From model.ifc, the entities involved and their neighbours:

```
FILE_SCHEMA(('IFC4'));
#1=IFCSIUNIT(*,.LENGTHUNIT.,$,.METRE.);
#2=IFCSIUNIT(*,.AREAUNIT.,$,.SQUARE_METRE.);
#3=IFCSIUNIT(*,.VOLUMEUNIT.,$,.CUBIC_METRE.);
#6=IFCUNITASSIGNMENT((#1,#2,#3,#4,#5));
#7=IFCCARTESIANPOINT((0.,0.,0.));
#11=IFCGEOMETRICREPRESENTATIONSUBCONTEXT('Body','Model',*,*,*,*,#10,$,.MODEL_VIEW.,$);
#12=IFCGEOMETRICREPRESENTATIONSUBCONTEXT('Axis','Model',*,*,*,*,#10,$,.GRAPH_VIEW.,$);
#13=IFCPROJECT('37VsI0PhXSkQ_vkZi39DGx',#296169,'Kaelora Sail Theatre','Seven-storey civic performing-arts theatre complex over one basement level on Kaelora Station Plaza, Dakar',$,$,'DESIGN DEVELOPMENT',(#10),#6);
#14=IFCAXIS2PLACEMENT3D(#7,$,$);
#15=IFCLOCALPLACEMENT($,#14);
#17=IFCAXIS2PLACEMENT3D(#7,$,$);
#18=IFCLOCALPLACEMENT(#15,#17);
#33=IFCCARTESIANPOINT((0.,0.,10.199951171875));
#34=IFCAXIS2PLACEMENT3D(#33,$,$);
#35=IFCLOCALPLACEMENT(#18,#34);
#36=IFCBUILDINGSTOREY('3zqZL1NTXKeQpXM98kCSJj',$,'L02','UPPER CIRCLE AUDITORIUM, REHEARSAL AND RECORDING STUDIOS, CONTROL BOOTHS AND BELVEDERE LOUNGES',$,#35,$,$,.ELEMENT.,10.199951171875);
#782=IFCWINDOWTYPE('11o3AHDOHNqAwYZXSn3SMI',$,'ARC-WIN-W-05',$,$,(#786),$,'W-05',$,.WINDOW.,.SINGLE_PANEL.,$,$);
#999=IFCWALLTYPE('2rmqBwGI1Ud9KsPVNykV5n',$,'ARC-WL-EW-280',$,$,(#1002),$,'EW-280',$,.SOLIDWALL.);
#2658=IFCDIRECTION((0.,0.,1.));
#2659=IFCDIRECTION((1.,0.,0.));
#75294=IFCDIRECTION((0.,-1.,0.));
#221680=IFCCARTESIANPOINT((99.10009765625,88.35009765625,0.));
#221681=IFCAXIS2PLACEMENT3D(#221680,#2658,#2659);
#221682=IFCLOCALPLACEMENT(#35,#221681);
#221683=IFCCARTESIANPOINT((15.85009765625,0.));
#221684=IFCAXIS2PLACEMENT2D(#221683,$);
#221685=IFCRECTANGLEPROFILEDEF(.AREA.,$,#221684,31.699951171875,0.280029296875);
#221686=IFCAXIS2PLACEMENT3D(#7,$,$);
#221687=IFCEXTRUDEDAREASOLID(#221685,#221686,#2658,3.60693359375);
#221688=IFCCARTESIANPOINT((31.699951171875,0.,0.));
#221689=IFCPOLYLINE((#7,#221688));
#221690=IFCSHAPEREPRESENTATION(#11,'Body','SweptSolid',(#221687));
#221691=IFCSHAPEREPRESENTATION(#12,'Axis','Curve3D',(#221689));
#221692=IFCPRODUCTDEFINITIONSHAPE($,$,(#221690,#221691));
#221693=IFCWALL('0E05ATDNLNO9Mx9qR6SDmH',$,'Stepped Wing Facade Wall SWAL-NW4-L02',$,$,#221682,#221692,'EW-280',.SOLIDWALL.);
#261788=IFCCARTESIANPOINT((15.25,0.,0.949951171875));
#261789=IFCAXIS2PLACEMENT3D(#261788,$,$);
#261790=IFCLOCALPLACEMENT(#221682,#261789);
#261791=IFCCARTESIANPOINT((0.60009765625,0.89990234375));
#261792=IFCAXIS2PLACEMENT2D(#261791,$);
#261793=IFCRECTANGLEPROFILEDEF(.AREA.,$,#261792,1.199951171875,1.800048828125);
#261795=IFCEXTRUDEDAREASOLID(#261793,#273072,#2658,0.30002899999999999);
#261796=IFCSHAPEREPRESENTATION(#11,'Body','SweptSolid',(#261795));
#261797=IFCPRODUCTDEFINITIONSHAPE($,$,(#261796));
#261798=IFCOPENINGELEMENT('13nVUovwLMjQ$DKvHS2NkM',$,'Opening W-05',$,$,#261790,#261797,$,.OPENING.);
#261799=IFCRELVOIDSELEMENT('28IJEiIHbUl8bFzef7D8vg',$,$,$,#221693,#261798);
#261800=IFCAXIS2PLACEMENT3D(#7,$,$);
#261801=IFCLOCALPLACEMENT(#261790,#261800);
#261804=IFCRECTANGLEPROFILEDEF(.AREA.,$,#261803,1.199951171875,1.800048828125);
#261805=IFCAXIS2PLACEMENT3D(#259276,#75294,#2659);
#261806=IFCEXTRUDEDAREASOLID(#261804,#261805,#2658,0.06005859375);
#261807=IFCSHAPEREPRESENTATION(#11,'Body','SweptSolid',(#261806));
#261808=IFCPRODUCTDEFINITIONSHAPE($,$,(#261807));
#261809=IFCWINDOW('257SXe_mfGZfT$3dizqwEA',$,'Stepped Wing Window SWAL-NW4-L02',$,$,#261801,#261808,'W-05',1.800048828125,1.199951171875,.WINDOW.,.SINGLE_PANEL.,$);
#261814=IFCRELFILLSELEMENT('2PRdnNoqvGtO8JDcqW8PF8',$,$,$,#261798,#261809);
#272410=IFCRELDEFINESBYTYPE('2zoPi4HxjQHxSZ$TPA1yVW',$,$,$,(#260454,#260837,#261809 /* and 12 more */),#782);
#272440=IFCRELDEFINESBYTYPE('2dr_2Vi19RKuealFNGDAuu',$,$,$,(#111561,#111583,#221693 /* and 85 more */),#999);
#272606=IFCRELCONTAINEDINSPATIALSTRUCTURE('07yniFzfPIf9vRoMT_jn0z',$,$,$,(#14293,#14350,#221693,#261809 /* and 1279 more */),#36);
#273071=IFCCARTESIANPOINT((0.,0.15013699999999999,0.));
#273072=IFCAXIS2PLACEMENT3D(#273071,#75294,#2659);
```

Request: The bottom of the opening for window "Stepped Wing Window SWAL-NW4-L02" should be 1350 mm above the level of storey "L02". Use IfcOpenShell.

```python
import numpy as np
import ifcopenshell
import ifcopenshell.api.geometry
import ifcopenshell.geom
import ifcopenshell.util.element
import ifcopenshell.util.placement
import ifcopenshell.util.shape
import ifcopenshell.util.unit

model = ifcopenshell.open("model.ifc")
unit_scale = ifcopenshell.util.unit.calculate_unit_scale(model)

window = model.by_guid("257SXe_mfGZfT$3dizqwEA")
opening = window.FillsVoids[0].RelatingOpeningElement
storey = ifcopenshell.util.element.get_container(window, ifc_class="IfcBuildingStorey")
level = ifcopenshell.util.placement.get_local_placement(storey.ObjectPlacement)[2, 3]

# The opening's origin need not be at the sill, so measure its lowest point.
shape = ifcopenshell.geom.create_shape(ifcopenshell.geom.settings(), opening)
bottom = ifcopenshell.util.shape.get_shape_bottom_elevation(shape, shape.geometry) / unit_scale
dz = level + 1.35 - bottom

shift = np.array([0.0, 0.0, dz])
# The window is placed relative to its opening, so it follows when the opening moves.
matrix = ifcopenshell.util.placement.get_local_placement(opening.ObjectPlacement)
matrix[:3, 3] += shift
ifcopenshell.api.geometry.edit_object_placement(
    model, product=opening, matrix=matrix, is_si=False, should_transform_children=True
)

print(f"moved by {dz * unit_scale:+.3f} m")

model.write("model-out.ifc")
```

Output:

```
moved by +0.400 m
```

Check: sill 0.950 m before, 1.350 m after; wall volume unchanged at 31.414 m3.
